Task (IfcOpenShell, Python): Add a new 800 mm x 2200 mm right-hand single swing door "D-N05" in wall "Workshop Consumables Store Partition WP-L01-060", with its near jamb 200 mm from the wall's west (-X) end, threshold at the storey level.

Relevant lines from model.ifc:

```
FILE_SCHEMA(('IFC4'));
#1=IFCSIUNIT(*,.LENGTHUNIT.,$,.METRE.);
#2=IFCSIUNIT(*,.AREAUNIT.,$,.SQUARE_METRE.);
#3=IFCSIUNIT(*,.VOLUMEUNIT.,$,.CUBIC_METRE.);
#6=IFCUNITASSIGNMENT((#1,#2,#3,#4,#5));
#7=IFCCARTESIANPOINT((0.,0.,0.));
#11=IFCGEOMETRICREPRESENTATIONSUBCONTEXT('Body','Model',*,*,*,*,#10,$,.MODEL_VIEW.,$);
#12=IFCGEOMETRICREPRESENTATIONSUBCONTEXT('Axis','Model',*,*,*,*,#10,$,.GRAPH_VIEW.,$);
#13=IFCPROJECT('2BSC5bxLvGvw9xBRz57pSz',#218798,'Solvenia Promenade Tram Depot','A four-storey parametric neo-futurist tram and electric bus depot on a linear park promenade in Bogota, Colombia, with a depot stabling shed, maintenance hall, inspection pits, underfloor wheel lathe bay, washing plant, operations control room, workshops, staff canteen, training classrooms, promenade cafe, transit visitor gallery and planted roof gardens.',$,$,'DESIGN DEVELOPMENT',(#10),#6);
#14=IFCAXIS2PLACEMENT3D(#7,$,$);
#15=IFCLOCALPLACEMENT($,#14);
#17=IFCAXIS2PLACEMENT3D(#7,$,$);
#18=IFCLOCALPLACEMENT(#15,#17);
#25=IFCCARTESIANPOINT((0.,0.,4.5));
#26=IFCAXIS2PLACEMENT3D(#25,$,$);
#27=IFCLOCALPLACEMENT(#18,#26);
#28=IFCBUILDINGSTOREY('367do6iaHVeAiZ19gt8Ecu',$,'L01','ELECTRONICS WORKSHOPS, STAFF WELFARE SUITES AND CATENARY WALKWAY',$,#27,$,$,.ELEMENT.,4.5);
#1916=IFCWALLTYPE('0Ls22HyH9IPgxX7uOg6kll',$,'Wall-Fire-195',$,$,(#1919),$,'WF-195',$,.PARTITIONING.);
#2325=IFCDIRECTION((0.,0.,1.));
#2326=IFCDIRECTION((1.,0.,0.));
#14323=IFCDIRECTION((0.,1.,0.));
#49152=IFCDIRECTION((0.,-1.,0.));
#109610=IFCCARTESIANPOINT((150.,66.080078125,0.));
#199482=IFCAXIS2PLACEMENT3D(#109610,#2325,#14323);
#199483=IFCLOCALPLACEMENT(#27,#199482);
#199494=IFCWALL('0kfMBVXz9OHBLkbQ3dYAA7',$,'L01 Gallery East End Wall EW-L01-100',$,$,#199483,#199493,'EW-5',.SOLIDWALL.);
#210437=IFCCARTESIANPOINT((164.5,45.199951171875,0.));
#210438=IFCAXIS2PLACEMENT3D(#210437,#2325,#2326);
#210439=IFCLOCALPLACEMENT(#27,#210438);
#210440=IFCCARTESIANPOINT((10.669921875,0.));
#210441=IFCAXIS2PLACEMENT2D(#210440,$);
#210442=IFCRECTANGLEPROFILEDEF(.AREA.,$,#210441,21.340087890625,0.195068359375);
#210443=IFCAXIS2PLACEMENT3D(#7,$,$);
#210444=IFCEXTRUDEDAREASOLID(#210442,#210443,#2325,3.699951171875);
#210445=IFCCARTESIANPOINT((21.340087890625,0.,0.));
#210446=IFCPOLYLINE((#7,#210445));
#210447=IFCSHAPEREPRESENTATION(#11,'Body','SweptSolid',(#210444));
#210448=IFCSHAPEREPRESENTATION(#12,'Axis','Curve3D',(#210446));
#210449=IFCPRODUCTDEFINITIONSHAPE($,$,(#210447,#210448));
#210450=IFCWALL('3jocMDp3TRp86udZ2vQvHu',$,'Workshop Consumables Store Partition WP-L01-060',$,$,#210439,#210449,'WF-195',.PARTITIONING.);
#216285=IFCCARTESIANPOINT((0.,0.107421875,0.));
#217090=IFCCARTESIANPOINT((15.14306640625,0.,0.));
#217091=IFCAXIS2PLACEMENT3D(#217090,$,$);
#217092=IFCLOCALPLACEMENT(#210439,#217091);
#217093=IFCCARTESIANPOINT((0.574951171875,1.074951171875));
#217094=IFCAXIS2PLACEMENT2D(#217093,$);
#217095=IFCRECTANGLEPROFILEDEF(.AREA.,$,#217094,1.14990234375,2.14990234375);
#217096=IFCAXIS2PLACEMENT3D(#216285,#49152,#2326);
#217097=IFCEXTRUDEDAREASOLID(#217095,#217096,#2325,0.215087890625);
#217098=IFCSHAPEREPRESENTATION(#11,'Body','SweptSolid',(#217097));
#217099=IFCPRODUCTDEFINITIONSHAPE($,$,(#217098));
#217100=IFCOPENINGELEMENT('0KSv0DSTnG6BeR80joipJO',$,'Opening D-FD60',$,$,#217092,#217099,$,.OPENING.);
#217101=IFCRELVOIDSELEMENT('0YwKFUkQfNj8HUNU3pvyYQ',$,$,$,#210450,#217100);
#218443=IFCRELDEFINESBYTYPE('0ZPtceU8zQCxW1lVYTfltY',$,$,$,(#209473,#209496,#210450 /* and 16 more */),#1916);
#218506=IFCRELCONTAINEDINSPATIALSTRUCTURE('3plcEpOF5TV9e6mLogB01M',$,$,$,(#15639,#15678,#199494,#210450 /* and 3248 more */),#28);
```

```python
import numpy as np
import ifcopenshell
import ifcopenshell.api.feature
import ifcopenshell.api.geometry
import ifcopenshell.api.root
import ifcopenshell.api.spatial
import ifcopenshell.geom
import ifcopenshell.util.element
import ifcopenshell.util.placement
import ifcopenshell.util.representation
import ifcopenshell.util.shape
import ifcopenshell.util.unit

model = ifcopenshell.open("model.ifc")
unit_scale = ifcopenshell.util.unit.calculate_unit_scale(model)
settings = ifcopenshell.geom.settings()


def volume(element):
    """Net volume in cubic metres, openings subtracted."""
    shape = ifcopenshell.geom.create_shape(settings, element)
    return ifcopenshell.util.shape.get_volume(shape.geometry)


wall = model.by_guid("3jocMDp3TRp86udZ2vQvHu")
storey = ifcopenshell.util.element.get_container(wall, ifc_class="IfcBuildingStorey")
context = ifcopenshell.util.representation.get_context(model, "Model", "Body", "MODEL_VIEW")
before = volume(wall)

width, height, from_end, sill = 0.8, 2.2, 0.2, 0.0  # metres

# The wall runs along its own X axis, and the end named is its -X end.
wall_shape = ifcopenshell.geom.create_shape(settings, wall)
x, y, z = ifcopenshell.util.shape.get_vertices(wall_shape.geometry).T
start = x.min() + from_end
face, thickness = float(y.min()), float(y.max() - y.min())
wall_matrix = ifcopenshell.util.placement.get_local_placement(wall.ObjectPlacement)
level = ifcopenshell.util.placement.get_local_placement(storey.ObjectPlacement)[2, 3]


def in_wall(x, y):
    """Placement at x, y metres in the wall's axes, at sill height."""
    matrix = wall_matrix.copy()
    matrix[:, 3] = wall_matrix @ np.array([x / unit_scale, y / unit_scale, 0.0, 1.0])
    matrix[2, 3] = level + sill / unit_scale
    return matrix


# Opening: a box that overshoots both wall faces by 50 mm.
opening = ifcopenshell.api.root.create_entity(model, ifc_class="IfcOpeningElement", predefined_type="OPENING")
box = ifcopenshell.api.geometry.add_wall_representation(
    model, context=context, length=width, height=height, thickness=thickness + 0.1
)
ifcopenshell.api.geometry.assign_representation(model, product=opening, representation=box)
ifcopenshell.api.geometry.edit_object_placement(model, product=opening, matrix=in_wall(start, face - 0.05), is_si=False)
ifcopenshell.api.feature.add_feature(model, feature=opening, element=wall)

door = ifcopenshell.api.root.create_entity(model, ifc_class="IfcDoor", name="D-N05", predefined_type="DOOR")
door.OverallWidth, door.OverallHeight = width / unit_scale, height / unit_scale
door.OperationType = "SINGLE_SWING_RIGHT"
body = ifcopenshell.api.geometry.add_door_representation(
    model,
    context=context,
    overall_width=door.OverallWidth,
    overall_height=door.OverallHeight,
    operation_type="SINGLE_SWING_RIGHT",
    lining_properties={"LiningDepth": thickness / unit_scale, "ThresholdDepth": thickness / unit_scale},
)
ifcopenshell.api.geometry.assign_representation(model, product=door, representation=body)
ifcopenshell.api.spatial.assign_container(model, products=[door], relating_structure=storey)
ifcopenshell.api.feature.add_filling(model, opening=opening, element=door)

# The lining spans the wall, so the door starts at the wall face.
ifcopenshell.api.geometry.edit_object_placement(model, product=door, matrix=in_wall(start, face), is_si=False)

after = volume(wall)

print(f"wall volume {before:.3f} -> {after:.3f} m3")

model.write("model-out.ifc")
```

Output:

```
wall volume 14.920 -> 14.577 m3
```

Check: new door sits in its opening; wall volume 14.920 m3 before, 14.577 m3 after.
